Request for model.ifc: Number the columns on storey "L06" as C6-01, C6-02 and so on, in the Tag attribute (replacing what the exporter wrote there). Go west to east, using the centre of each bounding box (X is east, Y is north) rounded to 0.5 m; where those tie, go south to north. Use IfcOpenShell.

First a look at what the model holds.

```python
import ifcopenshell
import ifcopenshell.util.element
import ifcopenshell.util.placement

model = ifcopenshell.open("model.ifc")
print(model.schema)
storey = next(s for s in model.by_type("IfcBuildingStorey") if s.Name == "L06")
columns = [e for e in ifcopenshell.util.element.get_decomposition(storey) if e.is_a("IfcColumn")]
for e in sorted(columns, key=lambda e: e.id()):
    origin = ifcopenshell.util.placement.get_local_placement(e.ObjectPlacement)[:3, 3]
    print(e.id(), e.Tag, e.Name, origin.round(2) + 0.0, sep=" | ")
```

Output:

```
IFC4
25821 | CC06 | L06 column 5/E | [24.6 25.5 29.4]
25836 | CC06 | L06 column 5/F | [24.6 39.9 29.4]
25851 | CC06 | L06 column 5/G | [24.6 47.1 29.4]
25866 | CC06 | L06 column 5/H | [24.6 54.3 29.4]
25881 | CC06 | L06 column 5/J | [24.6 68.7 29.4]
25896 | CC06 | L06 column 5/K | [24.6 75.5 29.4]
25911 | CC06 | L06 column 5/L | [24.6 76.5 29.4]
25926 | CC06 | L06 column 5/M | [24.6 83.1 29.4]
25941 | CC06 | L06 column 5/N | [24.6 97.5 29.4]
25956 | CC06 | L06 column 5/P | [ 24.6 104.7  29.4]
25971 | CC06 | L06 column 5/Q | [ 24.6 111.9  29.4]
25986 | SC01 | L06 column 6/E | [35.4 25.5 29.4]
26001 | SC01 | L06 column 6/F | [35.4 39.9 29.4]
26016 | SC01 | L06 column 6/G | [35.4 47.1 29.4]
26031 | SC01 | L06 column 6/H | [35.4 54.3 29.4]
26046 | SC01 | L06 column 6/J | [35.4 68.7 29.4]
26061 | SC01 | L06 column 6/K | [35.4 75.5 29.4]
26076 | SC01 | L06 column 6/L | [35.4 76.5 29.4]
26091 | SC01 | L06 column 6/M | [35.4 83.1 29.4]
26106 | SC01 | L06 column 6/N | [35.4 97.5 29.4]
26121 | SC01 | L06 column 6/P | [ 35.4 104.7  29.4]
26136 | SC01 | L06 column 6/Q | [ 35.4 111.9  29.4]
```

```python
import ifcopenshell
import ifcopenshell.geom
import ifcopenshell.util.element
import ifcopenshell.util.shape

model = ifcopenshell.open("model.ifc")
settings = ifcopenshell.geom.settings()
settings.set("use-world-coords", True)


def centre(element):
    shape = ifcopenshell.geom.create_shape(settings, element)
    return ifcopenshell.util.shape.get_bbox_centroid(shape.geometry)


storey = next(s for s in model.by_type("IfcBuildingStorey") if s.Name == "L06")
columns = [e for e in ifcopenshell.util.element.get_decomposition(storey) if e.is_a("IfcColumn")]

# Insertion points can sit at a corner or the storey origin, so sort by the geometry (in metres).
centres = {e: centre(e) for e in columns}
columns.sort(key=lambda e: (round(centres[e][0] / 0.5), centres[e][1]))

for i, e in enumerate(columns, start=1):
    number = f"C6-{i:02d}"
    e.Tag = number
    print(e.id(), number)

model.write("model_rev.ifc")
```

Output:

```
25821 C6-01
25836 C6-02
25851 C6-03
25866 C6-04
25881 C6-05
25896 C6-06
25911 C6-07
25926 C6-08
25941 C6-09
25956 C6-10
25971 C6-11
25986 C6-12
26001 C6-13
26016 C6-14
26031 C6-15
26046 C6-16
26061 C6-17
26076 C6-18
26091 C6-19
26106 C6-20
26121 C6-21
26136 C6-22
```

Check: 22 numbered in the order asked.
